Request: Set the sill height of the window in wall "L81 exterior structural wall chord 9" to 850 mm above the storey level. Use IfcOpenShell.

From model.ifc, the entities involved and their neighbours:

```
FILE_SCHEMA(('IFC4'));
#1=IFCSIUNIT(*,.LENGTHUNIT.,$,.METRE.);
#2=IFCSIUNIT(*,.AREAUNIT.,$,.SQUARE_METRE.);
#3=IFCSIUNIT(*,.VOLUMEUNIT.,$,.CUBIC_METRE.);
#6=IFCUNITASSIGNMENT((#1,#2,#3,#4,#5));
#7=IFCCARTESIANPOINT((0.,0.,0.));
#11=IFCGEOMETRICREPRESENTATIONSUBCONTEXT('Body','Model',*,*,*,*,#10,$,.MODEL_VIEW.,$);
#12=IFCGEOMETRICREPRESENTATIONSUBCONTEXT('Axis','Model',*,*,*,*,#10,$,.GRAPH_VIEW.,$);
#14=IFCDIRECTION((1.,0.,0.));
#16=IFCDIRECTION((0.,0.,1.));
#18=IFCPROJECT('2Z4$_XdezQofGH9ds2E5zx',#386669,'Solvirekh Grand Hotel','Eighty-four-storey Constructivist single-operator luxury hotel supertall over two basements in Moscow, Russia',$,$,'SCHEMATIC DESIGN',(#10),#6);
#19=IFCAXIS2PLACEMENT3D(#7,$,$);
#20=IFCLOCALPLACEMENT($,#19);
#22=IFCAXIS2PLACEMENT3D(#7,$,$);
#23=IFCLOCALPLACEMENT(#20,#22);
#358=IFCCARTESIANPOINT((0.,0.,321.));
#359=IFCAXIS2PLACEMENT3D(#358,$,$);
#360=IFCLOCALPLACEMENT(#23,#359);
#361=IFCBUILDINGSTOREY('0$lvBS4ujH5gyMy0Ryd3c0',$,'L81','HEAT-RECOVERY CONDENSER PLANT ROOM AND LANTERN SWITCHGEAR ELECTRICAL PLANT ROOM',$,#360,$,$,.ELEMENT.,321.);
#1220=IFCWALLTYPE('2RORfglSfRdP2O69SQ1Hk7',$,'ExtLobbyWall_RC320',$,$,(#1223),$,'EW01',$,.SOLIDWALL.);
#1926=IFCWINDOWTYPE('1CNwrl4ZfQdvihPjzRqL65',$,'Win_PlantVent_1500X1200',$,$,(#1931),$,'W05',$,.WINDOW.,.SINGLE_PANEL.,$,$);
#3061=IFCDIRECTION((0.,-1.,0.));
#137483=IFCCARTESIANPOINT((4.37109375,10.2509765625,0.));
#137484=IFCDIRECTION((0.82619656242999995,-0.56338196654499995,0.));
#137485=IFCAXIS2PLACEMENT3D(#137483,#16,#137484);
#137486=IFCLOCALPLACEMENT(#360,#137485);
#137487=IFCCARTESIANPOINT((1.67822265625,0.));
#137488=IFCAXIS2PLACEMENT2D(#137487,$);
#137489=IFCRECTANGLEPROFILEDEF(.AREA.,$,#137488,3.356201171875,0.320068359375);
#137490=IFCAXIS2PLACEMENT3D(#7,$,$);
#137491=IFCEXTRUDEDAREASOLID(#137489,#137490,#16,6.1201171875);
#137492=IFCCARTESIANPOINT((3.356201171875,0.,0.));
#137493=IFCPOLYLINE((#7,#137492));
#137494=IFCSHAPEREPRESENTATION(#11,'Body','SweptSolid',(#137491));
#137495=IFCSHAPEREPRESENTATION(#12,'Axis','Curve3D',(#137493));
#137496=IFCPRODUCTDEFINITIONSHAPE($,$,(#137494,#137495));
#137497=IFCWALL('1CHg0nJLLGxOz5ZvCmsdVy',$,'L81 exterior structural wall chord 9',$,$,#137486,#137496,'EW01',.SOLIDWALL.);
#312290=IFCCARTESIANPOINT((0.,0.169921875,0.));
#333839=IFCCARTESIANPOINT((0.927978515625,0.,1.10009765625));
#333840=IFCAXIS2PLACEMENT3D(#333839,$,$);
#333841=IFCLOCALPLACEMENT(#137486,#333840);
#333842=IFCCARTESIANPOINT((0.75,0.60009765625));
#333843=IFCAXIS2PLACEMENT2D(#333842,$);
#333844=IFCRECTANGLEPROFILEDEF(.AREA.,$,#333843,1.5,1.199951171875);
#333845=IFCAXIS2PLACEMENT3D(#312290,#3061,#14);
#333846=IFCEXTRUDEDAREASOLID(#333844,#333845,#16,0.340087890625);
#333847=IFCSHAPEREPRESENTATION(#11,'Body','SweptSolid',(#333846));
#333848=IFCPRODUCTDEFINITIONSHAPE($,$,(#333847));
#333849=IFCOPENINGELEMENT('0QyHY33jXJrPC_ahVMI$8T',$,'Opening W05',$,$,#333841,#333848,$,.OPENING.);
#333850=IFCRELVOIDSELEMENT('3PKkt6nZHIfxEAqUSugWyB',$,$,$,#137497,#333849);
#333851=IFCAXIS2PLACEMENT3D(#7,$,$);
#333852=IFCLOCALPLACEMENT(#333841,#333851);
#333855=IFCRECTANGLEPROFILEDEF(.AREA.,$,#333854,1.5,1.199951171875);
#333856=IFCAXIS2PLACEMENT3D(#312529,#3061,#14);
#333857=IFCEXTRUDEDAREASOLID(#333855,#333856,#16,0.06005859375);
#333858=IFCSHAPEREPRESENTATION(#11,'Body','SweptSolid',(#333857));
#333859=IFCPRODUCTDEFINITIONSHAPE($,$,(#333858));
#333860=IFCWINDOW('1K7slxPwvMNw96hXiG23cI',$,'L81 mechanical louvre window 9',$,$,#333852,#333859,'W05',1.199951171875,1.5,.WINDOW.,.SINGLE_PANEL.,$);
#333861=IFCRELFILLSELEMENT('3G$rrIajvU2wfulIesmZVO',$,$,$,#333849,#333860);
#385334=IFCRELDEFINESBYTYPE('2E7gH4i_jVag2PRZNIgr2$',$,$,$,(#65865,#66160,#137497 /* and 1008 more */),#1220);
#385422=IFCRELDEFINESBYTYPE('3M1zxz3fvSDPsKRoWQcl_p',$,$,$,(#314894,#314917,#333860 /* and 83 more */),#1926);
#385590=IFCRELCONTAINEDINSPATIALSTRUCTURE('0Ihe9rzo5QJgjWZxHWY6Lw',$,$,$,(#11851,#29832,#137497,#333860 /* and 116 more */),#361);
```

```python
import numpy as np
import ifcopenshell
import ifcopenshell.api.geometry
import ifcopenshell.geom
import ifcopenshell.util.element
import ifcopenshell.util.placement
import ifcopenshell.util.shape
import ifcopenshell.util.unit

model = ifcopenshell.open("model.ifc")
unit_scale = ifcopenshell.util.unit.calculate_unit_scale(model)

window = model.by_guid("1K7slxPwvMNw96hXiG23cI")
opening = window.FillsVoids[0].RelatingOpeningElement
storey = ifcopenshell.util.element.get_container(window, ifc_class="IfcBuildingStorey")
level = ifcopenshell.util.placement.get_local_placement(storey.ObjectPlacement)[2, 3]

# The opening's origin need not be at the sill, so measure its lowest point.
shape = ifcopenshell.geom.create_shape(ifcopenshell.geom.settings(), opening)
bottom = ifcopenshell.util.shape.get_shape_bottom_elevation(shape, shape.geometry) / unit_scale
dz = level + 0.85 / unit_scale - bottom

shift = np.array([0.0, 0.0, dz])
# The window is placed relative to its opening, so it follows when the opening moves.
matrix = ifcopenshell.util.placement.get_local_placement(opening.ObjectPlacement)
matrix[:3, 3] += shift
ifcopenshell.api.geometry.edit_object_placement(
    model, product=opening, matrix=matrix, is_si=False, should_transform_children=True
)

print(f"moved by {dz * unit_scale:+.3f} m")

model.write("model_rev.ifc")
```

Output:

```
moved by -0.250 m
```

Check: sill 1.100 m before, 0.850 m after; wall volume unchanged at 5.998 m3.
